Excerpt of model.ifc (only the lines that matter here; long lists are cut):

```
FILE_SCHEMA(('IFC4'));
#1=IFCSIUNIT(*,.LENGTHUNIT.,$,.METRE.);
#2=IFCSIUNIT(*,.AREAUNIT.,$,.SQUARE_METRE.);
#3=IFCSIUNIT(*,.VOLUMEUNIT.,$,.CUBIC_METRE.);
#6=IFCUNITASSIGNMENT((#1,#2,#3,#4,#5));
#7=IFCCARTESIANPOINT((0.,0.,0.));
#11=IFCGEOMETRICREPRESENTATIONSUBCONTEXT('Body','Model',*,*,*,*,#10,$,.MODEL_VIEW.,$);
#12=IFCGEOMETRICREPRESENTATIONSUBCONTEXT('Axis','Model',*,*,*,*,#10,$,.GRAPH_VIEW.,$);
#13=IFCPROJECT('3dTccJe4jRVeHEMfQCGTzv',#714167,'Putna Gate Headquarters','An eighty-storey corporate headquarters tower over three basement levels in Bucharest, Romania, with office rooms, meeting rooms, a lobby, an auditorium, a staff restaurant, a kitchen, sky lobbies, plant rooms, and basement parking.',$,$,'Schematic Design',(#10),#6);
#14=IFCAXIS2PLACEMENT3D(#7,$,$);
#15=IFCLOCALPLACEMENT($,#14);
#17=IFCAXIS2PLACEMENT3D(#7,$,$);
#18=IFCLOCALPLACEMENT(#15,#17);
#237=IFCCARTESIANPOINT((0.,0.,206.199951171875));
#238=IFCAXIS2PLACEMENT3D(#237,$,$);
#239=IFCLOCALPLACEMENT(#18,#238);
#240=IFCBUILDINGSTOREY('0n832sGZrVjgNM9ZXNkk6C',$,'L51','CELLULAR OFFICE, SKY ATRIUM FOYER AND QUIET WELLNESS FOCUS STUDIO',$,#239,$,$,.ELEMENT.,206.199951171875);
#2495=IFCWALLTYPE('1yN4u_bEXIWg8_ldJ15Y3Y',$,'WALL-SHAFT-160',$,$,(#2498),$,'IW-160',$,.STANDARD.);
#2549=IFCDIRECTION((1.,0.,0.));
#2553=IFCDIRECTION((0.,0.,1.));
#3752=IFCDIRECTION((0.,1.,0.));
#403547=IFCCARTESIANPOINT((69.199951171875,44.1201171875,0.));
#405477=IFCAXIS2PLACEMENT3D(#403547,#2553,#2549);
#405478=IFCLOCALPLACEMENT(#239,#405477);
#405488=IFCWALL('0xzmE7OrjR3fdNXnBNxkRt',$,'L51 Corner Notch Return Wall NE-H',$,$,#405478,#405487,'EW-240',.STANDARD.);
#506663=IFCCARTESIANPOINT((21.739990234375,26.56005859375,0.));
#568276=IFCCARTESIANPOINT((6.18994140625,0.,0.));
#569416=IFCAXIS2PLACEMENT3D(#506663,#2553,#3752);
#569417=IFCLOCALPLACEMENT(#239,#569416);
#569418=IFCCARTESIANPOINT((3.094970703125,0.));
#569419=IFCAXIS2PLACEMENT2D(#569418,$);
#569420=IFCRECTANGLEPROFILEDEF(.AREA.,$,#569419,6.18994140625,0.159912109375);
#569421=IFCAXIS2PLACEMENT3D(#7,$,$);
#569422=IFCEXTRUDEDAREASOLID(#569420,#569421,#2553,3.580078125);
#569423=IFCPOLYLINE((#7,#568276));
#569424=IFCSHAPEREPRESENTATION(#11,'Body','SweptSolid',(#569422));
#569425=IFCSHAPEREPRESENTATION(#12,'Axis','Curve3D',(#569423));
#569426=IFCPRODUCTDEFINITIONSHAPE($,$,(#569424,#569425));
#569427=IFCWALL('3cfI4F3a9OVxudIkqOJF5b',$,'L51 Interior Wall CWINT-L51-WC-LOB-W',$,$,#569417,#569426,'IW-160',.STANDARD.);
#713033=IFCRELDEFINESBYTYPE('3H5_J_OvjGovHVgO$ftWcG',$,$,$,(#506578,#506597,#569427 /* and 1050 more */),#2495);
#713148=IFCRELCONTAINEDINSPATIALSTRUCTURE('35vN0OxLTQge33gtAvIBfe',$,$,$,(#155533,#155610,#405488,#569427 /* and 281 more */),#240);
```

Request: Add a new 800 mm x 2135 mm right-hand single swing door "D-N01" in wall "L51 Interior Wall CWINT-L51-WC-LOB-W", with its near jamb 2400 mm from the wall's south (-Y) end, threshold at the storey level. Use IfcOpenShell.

```python
import numpy as np
import ifcopenshell
import ifcopenshell.api.feature
import ifcopenshell.api.geometry
import ifcopenshell.api.root
import ifcopenshell.api.spatial
import ifcopenshell.geom
import ifcopenshell.util.element
import ifcopenshell.util.placement
import ifcopenshell.util.representation
import ifcopenshell.util.shape
import ifcopenshell.util.unit

model = ifcopenshell.open("model.ifc")
unit_scale = ifcopenshell.util.unit.calculate_unit_scale(model)
settings = ifcopenshell.geom.settings()


def volume(element):
    """Net volume in cubic metres, openings subtracted."""
    shape = ifcopenshell.geom.create_shape(settings, element)
    return ifcopenshell.util.shape.get_volume(shape.geometry)


wall = model.by_id(569427)
storey = ifcopenshell.util.element.get_container(wall, ifc_class="IfcBuildingStorey")
context = ifcopenshell.util.representation.get_context(model, "Model", "Body", "MODEL_VIEW")
before = volume(wall)

width, height, from_end, sill = 0.8, 2.135, 2.4, 0.0  # metres

# The wall runs along its own X axis, and the end named is its -X end.
wall_shape = ifcopenshell.geom.create_shape(settings, wall)
x, y, z = ifcopenshell.util.shape.get_vertices(wall_shape.geometry).T
start = x.min() + from_end
face, thickness = float(y.min()), float(y.max() - y.min())
wall_matrix = ifcopenshell.util.placement.get_local_placement(wall.ObjectPlacement)
level = ifcopenshell.util.placement.get_local_placement(storey.ObjectPlacement)[2, 3]


def in_wall(x, y):
    """Placement at x, y metres in the wall's axes, at sill height."""
    matrix = wall_matrix.copy()
    matrix[:, 3] = wall_matrix @ np.array([x / unit_scale, y / unit_scale, 0.0, 1.0])
    matrix[2, 3] = level + sill / unit_scale
    return matrix


# Opening: a box that overshoots both wall faces by 50 mm.
opening = ifcopenshell.api.root.create_entity(model, ifc_class="IfcOpeningElement", predefined_type="OPENING")
box = ifcopenshell.api.geometry.add_wall_representation(
    model, context=context, length=width, height=height, thickness=thickness + 0.1
)
ifcopenshell.api.geometry.assign_representation(model, product=opening, representation=box)
ifcopenshell.api.geometry.edit_object_placement(model, product=opening, matrix=in_wall(start, face - 0.05), is_si=False)
ifcopenshell.api.feature.add_feature(model, feature=opening, element=wall)

door = ifcopenshell.api.root.create_entity(model, ifc_class="IfcDoor", name="D-N01", predefined_type="DOOR")
door.OverallWidth, door.OverallHeight = width / unit_scale, height / unit_scale
door.OperationType = "SINGLE_SWING_RIGHT"
body = ifcopenshell.api.geometry.add_door_representation(
    model,
    context=context,
    overall_width=door.OverallWidth,
    overall_height=door.OverallHeight,
    operation_type="SINGLE_SWING_RIGHT",
    lining_properties={"LiningDepth": thickness / unit_scale, "ThresholdDepth": thickness / unit_scale},
)
ifcopenshell.api.geometry.assign_representation(model, product=door, representation=body)
ifcopenshell.api.spatial.assign_container(model, products=[door], relating_structure=storey)
ifcopenshell.api.feature.add_filling(model, opening=opening, element=door)

# The lining spans the wall, so the door starts at the wall face.
ifcopenshell.api.geometry.edit_object_placement(model, product=door, matrix=in_wall(start, face), is_si=False)

after = volume(wall)

print(f"wall volume {before:.3f} -> {after:.3f} m3")

model.write("model_v2.ifc")
```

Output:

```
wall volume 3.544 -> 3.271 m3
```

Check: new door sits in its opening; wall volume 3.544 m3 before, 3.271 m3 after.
